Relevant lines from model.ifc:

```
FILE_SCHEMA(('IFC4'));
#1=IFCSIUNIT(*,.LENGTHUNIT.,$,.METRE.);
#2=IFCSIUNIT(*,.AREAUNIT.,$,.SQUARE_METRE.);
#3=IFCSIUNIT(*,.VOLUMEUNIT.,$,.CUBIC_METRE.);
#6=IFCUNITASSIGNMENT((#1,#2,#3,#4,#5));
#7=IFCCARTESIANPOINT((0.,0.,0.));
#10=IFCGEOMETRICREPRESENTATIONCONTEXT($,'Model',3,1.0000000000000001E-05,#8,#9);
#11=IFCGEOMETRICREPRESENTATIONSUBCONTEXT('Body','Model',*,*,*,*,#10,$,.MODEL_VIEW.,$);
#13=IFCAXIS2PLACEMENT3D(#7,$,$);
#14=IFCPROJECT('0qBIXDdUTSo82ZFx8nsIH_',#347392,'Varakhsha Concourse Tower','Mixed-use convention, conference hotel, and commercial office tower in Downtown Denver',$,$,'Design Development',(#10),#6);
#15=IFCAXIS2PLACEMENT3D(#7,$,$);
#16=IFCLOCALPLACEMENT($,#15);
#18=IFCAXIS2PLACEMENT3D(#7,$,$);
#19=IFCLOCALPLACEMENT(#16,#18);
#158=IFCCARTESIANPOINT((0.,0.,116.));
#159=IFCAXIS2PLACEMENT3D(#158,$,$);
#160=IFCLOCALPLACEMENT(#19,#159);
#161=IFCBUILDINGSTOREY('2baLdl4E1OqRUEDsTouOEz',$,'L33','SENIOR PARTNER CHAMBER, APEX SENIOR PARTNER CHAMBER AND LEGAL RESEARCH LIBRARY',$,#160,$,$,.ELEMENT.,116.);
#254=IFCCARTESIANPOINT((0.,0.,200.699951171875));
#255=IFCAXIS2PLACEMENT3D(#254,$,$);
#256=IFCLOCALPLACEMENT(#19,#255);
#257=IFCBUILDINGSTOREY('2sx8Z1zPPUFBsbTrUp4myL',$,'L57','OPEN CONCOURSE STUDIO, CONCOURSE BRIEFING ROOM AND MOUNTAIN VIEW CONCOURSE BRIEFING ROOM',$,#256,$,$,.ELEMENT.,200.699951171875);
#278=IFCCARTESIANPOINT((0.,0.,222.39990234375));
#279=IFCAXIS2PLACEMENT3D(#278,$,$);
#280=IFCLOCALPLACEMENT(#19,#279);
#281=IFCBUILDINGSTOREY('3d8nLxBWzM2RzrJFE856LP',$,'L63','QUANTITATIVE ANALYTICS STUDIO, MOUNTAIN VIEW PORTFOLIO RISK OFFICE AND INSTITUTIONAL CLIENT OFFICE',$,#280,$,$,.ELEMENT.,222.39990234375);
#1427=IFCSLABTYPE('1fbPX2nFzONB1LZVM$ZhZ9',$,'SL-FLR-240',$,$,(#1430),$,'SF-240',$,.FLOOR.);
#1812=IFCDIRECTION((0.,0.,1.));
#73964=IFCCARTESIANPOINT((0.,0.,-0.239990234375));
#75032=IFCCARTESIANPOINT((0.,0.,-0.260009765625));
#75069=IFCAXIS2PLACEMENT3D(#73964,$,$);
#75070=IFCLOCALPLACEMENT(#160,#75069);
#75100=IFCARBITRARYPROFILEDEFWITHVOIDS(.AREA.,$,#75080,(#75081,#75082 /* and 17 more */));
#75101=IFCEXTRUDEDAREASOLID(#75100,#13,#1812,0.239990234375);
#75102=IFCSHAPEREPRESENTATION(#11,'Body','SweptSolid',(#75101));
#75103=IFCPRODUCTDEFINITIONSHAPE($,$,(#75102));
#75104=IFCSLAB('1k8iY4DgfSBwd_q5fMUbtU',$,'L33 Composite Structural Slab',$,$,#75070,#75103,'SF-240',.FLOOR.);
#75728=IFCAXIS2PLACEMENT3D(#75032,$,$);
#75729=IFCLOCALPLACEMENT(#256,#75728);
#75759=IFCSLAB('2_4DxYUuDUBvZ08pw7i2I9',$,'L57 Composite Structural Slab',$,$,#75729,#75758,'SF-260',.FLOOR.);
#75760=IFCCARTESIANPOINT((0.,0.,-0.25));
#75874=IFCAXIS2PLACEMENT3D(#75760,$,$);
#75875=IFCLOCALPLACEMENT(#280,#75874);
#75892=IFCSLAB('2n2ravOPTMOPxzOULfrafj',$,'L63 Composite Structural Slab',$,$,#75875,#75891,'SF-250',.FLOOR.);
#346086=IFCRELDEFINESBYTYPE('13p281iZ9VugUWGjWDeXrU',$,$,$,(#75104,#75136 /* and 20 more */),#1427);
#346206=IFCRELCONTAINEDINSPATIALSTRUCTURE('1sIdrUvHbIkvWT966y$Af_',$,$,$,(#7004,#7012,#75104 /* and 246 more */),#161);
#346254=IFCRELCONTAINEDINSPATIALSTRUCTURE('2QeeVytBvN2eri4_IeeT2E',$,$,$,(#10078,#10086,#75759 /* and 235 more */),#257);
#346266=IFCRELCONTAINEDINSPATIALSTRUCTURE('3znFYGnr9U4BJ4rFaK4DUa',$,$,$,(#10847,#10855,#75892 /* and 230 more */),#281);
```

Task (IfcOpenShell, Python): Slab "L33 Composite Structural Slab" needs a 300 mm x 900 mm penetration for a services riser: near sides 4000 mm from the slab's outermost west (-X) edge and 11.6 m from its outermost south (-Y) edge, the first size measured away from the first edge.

```python
import numpy as np
import ifcopenshell
import ifcopenshell.api.feature
import ifcopenshell.api.geometry
import ifcopenshell.api.root
import ifcopenshell.geom
import ifcopenshell.util.placement
import ifcopenshell.util.representation
import ifcopenshell.util.shape
import ifcopenshell.util.unit

model = ifcopenshell.open("model.ifc")
unit_scale = ifcopenshell.util.unit.calculate_unit_scale(model)
settings = ifcopenshell.geom.settings()


def volume(element):
    """Net volume in cubic metres, openings subtracted."""
    shape = ifcopenshell.geom.create_shape(settings, element)
    return ifcopenshell.util.shape.get_volume(shape.geometry)


slab = model.by_guid("1k8iY4DgfSBwd_q5fMUbtU")
before = volume(slab)

# Extent in the slab's own axes, in metres. The edges named are its -X and -Y sides.
slab_shape = ifcopenshell.geom.create_shape(settings, slab)
vertices = ifcopenshell.util.shape.get_vertices(slab_shape.geometry)
x_min, y_min, bottom = vertices.min(axis=0)
top = vertices[:, 2].max()

opening = ifcopenshell.api.root.create_entity(model, ifc_class="IfcOpeningElement", name="Services riser opening", predefined_type="OPENING")
context = ifcopenshell.util.representation.get_context(model, "Model", "Body", "MODEL_VIEW")
width, depth = 0.3, 0.9
outline = [(0.0, 0.0), (width, 0.0), (width, depth), (0.0, depth), (0.0, 0.0)]
# Overshoot both faces by 50 mm so the cut is clean.
shape = ifcopenshell.api.geometry.add_slab_representation(
    model, context=context, depth=top - bottom + 0.1, polyline=outline
)
ifcopenshell.api.geometry.assign_representation(model, product=opening, representation=shape)

matrix = ifcopenshell.util.placement.get_local_placement(slab.ObjectPlacement)
matrix[:, 3] = matrix @ np.append(np.array([x_min + 4, y_min + 11.6, bottom - 0.05]) / unit_scale, 1.0)
ifcopenshell.api.geometry.edit_object_placement(model, product=opening, matrix=matrix, is_si=False)
ifcopenshell.api.feature.add_feature(model, feature=opening, element=slab)

after = volume(slab)

print(f"slab volume {before:.3f} -> {after:.3f} m3")

model.write("model_updated.ifc")
```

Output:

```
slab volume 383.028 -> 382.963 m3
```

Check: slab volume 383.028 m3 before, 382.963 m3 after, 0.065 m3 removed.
